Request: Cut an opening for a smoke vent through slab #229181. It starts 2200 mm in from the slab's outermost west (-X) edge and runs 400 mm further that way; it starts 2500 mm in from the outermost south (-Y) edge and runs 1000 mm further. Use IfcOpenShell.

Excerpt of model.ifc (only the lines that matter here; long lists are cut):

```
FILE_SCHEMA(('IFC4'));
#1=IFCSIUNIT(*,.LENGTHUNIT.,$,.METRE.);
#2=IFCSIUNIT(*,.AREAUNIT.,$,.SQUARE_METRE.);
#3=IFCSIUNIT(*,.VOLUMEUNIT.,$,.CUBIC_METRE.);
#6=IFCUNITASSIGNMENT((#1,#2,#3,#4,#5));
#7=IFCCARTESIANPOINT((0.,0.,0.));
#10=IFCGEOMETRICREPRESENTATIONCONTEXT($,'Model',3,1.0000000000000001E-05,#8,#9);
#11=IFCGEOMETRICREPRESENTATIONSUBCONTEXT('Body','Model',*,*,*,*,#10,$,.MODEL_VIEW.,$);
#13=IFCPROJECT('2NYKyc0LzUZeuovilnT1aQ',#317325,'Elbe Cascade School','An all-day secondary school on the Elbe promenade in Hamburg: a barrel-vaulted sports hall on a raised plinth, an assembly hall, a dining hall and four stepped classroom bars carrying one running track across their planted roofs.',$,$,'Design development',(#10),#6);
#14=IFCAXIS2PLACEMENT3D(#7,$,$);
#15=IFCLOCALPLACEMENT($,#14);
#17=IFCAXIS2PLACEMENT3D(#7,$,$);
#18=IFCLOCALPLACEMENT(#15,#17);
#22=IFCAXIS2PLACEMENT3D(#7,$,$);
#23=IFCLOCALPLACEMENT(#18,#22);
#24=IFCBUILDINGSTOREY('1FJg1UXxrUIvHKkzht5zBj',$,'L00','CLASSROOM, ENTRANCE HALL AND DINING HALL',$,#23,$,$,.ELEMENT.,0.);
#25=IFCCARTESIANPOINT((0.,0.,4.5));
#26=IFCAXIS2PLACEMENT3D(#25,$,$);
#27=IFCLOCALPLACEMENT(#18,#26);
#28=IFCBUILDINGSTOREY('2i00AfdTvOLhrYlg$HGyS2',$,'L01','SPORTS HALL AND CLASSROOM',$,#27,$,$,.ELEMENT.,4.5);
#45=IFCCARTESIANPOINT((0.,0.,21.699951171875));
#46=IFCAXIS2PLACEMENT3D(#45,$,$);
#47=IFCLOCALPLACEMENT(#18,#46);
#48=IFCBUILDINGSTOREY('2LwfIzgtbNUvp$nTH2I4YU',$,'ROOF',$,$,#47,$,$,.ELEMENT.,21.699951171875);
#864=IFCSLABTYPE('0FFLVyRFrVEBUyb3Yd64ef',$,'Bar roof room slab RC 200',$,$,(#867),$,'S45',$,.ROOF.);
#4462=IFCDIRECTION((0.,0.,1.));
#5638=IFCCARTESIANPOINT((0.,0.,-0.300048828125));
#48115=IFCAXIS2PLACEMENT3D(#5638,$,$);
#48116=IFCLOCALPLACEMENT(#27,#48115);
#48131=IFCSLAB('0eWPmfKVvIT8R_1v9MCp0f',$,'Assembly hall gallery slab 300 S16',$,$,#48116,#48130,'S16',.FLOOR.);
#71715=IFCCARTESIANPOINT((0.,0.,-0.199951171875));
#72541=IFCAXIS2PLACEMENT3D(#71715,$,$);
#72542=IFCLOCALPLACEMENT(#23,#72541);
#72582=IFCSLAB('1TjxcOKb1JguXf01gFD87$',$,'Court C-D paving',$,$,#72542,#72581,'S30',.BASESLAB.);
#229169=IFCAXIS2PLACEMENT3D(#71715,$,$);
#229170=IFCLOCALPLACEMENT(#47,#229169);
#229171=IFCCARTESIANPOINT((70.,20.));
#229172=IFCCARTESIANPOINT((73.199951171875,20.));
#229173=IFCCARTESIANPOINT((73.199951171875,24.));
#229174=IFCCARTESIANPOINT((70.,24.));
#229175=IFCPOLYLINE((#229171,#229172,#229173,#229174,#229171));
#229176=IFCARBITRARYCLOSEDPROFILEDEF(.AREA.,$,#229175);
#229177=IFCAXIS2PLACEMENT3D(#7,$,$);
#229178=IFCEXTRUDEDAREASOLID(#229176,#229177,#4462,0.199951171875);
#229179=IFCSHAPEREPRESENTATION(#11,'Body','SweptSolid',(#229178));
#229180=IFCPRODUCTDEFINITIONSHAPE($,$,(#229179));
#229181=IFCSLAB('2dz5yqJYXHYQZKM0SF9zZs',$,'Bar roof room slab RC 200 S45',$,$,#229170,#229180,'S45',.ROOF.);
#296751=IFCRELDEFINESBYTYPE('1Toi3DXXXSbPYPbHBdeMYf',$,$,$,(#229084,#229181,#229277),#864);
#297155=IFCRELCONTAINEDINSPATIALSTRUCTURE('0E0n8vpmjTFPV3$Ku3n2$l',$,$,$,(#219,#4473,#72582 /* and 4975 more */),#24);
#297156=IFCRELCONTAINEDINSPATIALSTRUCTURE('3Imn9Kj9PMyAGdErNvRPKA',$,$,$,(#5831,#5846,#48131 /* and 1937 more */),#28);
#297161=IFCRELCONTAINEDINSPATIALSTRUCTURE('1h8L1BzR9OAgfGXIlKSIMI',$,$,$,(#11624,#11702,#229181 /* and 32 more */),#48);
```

```python
import numpy as np
import ifcopenshell
import ifcopenshell.api.feature
import ifcopenshell.api.geometry
import ifcopenshell.api.root
import ifcopenshell.geom
import ifcopenshell.util.placement
import ifcopenshell.util.representation
import ifcopenshell.util.shape
import ifcopenshell.util.unit

model = ifcopenshell.open("model.ifc")
unit_scale = ifcopenshell.util.unit.calculate_unit_scale(model)
settings = ifcopenshell.geom.settings()


def volume(element):
    """Net volume in cubic metres, openings subtracted."""
    shape = ifcopenshell.geom.create_shape(settings, element)
    return ifcopenshell.util.shape.get_volume(shape.geometry)


slab = model.by_id(229181)
before = volume(slab)

# Extent in the slab's own axes, in metres. The edges named are its -X and -Y sides.
slab_shape = ifcopenshell.geom.create_shape(settings, slab)
vertices = ifcopenshell.util.shape.get_vertices(slab_shape.geometry)
x_min, y_min, bottom = vertices.min(axis=0)
top = vertices[:, 2].max()

opening = ifcopenshell.api.root.create_entity(model, ifc_class="IfcOpeningElement", name="Smoke vent opening", predefined_type="OPENING")
context = ifcopenshell.util.representation.get_context(model, "Model", "Body", "MODEL_VIEW")
width, depth = 0.4, 1
outline = [(0.0, 0.0), (width, 0.0), (width, depth), (0.0, depth), (0.0, 0.0)]
# Overshoot both faces by 50 mm so the cut is clean.
shape = ifcopenshell.api.geometry.add_slab_representation(
    model, context=context, depth=top - bottom + 0.1, polyline=outline
)
ifcopenshell.api.geometry.assign_representation(model, product=opening, representation=shape)

matrix = ifcopenshell.util.placement.get_local_placement(slab.ObjectPlacement)
matrix[:, 3] = matrix @ np.append(np.array([x_min + 2.2, y_min + 2.5, bottom - 0.05]) / unit_scale, 1.0)
ifcopenshell.api.geometry.edit_object_placement(model, product=opening, matrix=matrix, is_si=False)
ifcopenshell.api.feature.add_feature(model, feature=opening, element=slab)

after = volume(slab)

print(f"slab volume {before:.3f} -> {after:.3f} m3")

model.write("model_updated.ifc")
```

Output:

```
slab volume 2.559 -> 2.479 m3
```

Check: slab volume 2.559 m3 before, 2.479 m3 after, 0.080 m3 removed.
